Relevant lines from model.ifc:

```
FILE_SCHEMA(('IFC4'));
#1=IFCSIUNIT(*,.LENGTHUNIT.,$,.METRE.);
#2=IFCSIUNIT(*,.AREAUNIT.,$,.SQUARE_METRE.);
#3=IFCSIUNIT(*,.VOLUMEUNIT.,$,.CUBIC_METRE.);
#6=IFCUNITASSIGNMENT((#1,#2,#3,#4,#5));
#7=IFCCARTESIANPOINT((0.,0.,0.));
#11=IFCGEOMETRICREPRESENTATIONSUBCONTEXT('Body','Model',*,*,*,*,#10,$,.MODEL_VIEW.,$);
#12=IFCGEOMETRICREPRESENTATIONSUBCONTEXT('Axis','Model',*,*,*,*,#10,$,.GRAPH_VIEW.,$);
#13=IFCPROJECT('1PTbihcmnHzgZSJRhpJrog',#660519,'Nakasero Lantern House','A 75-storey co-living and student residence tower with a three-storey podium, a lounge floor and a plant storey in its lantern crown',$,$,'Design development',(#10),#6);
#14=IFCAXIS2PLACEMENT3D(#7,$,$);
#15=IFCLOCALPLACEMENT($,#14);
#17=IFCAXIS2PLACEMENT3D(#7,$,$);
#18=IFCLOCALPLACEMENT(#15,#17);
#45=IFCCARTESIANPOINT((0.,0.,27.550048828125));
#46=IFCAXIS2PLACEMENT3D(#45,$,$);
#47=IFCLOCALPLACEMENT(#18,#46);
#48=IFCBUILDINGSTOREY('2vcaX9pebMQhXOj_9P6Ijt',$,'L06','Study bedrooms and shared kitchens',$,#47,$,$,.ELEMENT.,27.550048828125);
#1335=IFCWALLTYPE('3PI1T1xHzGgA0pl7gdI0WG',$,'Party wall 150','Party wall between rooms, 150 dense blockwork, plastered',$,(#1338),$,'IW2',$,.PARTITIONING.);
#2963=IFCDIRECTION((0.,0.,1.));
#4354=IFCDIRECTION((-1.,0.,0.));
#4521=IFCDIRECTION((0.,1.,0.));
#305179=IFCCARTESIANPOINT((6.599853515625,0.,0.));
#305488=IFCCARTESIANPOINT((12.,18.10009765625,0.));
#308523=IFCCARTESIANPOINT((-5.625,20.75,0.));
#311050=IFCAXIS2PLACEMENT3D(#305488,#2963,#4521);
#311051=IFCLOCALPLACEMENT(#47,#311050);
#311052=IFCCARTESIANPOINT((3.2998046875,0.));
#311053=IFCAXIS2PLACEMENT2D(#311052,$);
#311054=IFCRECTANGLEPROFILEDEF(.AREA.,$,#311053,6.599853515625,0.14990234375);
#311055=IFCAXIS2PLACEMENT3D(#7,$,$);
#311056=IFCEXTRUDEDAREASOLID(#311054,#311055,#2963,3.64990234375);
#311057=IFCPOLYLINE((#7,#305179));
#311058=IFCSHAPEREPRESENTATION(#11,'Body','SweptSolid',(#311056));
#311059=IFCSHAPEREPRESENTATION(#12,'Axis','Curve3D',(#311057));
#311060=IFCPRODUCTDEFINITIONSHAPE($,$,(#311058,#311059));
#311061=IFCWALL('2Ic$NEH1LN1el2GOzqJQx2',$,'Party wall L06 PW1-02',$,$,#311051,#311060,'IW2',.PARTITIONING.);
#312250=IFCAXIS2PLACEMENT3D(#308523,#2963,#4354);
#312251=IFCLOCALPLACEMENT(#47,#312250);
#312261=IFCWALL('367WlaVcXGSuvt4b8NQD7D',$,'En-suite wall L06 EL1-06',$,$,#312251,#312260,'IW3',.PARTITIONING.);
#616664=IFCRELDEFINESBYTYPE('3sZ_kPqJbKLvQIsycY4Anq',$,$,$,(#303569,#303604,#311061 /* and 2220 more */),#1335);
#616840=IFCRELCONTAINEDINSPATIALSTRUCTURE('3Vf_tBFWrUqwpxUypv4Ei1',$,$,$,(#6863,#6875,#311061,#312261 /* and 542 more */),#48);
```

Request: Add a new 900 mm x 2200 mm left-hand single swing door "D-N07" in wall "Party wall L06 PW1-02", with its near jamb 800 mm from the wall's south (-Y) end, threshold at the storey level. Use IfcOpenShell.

```python
import numpy as np
import ifcopenshell
import ifcopenshell.api.feature
import ifcopenshell.api.geometry
import ifcopenshell.api.root
import ifcopenshell.api.spatial
import ifcopenshell.geom
import ifcopenshell.util.element
import ifcopenshell.util.placement
import ifcopenshell.util.representation
import ifcopenshell.util.shape
import ifcopenshell.util.unit

model = ifcopenshell.open("model.ifc")
unit_scale = ifcopenshell.util.unit.calculate_unit_scale(model)
settings = ifcopenshell.geom.settings()


def volume(element):
    """Net volume in cubic metres, openings subtracted."""
    shape = ifcopenshell.geom.create_shape(settings, element)
    return ifcopenshell.util.shape.get_volume(shape.geometry)


wall = model.by_guid("2Ic$NEH1LN1el2GOzqJQx2")
storey = ifcopenshell.util.element.get_container(wall, ifc_class="IfcBuildingStorey")
context = ifcopenshell.util.representation.get_context(model, "Model", "Body", "MODEL_VIEW")
before = volume(wall)

width, height, from_end, sill = 0.9, 2.2, 0.8, 0.0  # metres

# The wall runs along its own X axis, and the end named is its -X end.
wall_shape = ifcopenshell.geom.create_shape(settings, wall)
x, y, z = ifcopenshell.util.shape.get_vertices(wall_shape.geometry).T
start = x.min() + from_end
face, thickness = float(y.min()), float(y.max() - y.min())
wall_matrix = ifcopenshell.util.placement.get_local_placement(wall.ObjectPlacement)
level = ifcopenshell.util.placement.get_local_placement(storey.ObjectPlacement)[2, 3]


def in_wall(x, y):
    """Placement at x, y metres in the wall's axes, at sill height."""
    matrix = wall_matrix.copy()
    matrix[:, 3] = wall_matrix @ np.array([x / unit_scale, y / unit_scale, 0.0, 1.0])
    matrix[2, 3] = level + sill / unit_scale
    return matrix


# Opening: a box that overshoots both wall faces by 50 mm.
opening = ifcopenshell.api.root.create_entity(model, ifc_class="IfcOpeningElement", predefined_type="OPENING")
box = ifcopenshell.api.geometry.add_wall_representation(
    model, context=context, length=width, height=height, thickness=thickness + 0.1
)
ifcopenshell.api.geometry.assign_representation(model, product=opening, representation=box)
ifcopenshell.api.geometry.edit_object_placement(model, product=opening, matrix=in_wall(start, face - 0.05), is_si=False)
ifcopenshell.api.feature.add_feature(model, feature=opening, element=wall)

door = ifcopenshell.api.root.create_entity(model, ifc_class="IfcDoor", name="D-N07", predefined_type="DOOR")
door.OverallWidth, door.OverallHeight = width / unit_scale, height / unit_scale
door.OperationType = "SINGLE_SWING_LEFT"
body = ifcopenshell.api.geometry.add_door_representation(
    model,
    context=context,
    overall_width=door.OverallWidth,
    overall_height=door.OverallHeight,
    operation_type="SINGLE_SWING_LEFT",
    lining_properties={"LiningDepth": thickness / unit_scale, "ThresholdDepth": thickness / unit_scale},
)
ifcopenshell.api.geometry.assign_representation(model, product=door, representation=body)
ifcopenshell.api.spatial.assign_container(model, products=[door], relating_structure=storey)
ifcopenshell.api.feature.add_filling(model, opening=opening, element=door)

# The lining spans the wall, so the door starts at the wall face.
ifcopenshell.api.geometry.edit_object_placement(model, product=door, matrix=in_wall(start, face), is_si=False)

after = volume(wall)

print(f"wall volume {before:.3f} -> {after:.3f} m3")

model.write("model_v2.ifc")
```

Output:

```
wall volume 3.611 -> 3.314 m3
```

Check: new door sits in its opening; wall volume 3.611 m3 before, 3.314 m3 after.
